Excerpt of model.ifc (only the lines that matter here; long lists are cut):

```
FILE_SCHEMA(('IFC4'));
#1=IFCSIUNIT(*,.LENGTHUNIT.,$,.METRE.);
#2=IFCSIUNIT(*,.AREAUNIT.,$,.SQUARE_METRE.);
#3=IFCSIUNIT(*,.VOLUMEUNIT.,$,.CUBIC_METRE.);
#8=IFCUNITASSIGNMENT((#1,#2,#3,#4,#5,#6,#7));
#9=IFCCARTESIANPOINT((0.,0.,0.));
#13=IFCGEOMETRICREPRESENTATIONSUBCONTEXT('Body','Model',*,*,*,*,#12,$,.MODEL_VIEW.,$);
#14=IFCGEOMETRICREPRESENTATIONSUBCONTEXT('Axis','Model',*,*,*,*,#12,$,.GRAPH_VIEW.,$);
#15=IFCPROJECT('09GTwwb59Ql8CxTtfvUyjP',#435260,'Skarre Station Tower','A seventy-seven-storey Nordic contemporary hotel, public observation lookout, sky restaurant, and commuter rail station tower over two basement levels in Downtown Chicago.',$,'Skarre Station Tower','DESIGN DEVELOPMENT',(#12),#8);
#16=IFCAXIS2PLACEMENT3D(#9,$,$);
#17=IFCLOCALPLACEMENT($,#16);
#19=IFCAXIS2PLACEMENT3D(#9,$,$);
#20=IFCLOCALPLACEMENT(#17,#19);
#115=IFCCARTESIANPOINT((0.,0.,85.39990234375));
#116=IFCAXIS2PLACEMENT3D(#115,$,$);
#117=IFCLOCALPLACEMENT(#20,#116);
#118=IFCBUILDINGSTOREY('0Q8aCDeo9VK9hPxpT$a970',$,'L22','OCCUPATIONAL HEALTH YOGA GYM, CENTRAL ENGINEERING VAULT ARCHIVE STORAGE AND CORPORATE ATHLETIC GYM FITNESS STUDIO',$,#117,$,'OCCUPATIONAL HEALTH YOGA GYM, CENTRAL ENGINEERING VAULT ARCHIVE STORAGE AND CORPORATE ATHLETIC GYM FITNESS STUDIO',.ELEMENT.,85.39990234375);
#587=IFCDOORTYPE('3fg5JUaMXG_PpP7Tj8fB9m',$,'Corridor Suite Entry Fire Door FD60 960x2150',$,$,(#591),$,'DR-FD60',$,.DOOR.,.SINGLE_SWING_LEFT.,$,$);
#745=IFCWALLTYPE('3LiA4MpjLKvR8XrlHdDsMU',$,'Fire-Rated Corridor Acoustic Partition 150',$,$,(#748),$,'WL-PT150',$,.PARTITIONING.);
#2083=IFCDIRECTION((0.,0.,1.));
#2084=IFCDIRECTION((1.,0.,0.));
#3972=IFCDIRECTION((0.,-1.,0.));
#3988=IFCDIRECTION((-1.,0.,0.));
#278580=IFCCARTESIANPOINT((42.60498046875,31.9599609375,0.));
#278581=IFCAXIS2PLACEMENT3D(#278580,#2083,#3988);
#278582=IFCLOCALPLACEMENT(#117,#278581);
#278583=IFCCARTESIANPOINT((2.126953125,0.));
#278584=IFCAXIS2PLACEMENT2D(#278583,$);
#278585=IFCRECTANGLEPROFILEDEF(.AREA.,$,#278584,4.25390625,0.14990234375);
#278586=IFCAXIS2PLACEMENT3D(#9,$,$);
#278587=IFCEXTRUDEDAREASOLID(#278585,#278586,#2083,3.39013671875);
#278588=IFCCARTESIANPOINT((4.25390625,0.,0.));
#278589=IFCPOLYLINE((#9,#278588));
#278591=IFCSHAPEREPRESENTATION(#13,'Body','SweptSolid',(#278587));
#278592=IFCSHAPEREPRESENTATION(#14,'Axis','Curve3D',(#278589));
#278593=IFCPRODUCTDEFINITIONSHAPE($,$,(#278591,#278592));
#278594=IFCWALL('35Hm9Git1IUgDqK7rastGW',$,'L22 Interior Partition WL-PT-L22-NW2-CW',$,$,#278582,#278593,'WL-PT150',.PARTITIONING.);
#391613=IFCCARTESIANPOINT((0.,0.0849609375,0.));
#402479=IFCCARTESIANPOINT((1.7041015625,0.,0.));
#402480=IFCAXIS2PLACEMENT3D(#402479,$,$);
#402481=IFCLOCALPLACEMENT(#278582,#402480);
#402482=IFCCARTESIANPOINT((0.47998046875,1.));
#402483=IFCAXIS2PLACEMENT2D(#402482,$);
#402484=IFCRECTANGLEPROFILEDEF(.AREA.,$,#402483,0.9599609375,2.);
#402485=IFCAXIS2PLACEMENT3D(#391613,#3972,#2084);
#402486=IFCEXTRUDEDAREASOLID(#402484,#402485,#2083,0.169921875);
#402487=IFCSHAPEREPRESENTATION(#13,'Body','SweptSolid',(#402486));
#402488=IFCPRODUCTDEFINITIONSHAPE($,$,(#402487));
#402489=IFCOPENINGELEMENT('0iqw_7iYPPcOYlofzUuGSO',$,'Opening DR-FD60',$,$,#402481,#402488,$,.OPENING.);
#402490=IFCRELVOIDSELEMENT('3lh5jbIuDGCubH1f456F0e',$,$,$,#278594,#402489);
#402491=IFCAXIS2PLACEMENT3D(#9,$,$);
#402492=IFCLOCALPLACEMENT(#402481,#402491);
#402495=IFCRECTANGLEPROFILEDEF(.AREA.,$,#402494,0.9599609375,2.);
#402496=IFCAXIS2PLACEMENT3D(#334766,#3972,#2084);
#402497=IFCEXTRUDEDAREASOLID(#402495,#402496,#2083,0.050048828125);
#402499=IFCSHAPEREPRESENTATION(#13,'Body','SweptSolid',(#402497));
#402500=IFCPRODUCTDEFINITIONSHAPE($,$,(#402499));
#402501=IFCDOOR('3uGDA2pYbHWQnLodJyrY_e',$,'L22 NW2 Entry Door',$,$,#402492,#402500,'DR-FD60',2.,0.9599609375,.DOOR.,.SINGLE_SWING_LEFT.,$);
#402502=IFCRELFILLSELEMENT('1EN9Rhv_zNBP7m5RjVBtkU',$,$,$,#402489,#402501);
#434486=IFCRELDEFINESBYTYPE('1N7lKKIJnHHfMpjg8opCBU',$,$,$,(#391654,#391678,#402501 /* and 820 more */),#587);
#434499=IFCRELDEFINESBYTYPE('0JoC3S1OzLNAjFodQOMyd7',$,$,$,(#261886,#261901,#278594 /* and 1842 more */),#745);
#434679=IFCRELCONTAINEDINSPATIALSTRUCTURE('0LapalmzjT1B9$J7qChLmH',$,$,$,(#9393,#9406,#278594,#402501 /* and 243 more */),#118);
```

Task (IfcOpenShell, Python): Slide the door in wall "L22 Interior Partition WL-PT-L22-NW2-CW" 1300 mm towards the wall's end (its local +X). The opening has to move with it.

```python
import ifcopenshell
import ifcopenshell.api.geometry
import ifcopenshell.util.placement
import ifcopenshell.util.unit

model = ifcopenshell.open("model.ifc")
unit_scale = ifcopenshell.util.unit.calculate_unit_scale(model)

door = model.by_guid("3uGDA2pYbHWQnLodJyrY_e")
opening = door.FillsVoids[0].RelatingOpeningElement
wall = opening.VoidsElements[0].RelatingBuildingElement

wall_matrix = ifcopenshell.util.placement.get_local_placement(wall.ObjectPlacement)
shift = wall_matrix[:3, 0] * 1.3 / unit_scale
before = ifcopenshell.util.placement.get_local_placement(door.ObjectPlacement)[:3, 3].copy()

# The door is placed relative to its opening, so it follows when the opening moves.
matrix = ifcopenshell.util.placement.get_local_placement(opening.ObjectPlacement)
matrix[:3, 3] += shift
ifcopenshell.api.geometry.edit_object_placement(
    model, product=opening, matrix=matrix, is_si=False, should_transform_children=True
)

after = ifcopenshell.util.placement.get_local_placement(door.ObjectPlacement)[:3, 3]
print("door moved by", (after - before).round(3) + 0.0)

model.write("model_edited.ifc")
```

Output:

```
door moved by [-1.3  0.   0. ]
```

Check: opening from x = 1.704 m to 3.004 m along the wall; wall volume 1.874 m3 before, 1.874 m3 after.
